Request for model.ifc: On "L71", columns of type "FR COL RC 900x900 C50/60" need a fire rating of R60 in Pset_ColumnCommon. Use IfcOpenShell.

First a look at what the model holds.

```python
import ifcopenshell
import ifcopenshell.util.element

model = ifcopenshell.open("model.ifc")
print(model.schema)
storey = next(s for s in model.by_type("IfcBuildingStorey") if s.Name == "L71")
columns = [e for e in ifcopenshell.util.element.get_decomposition(storey) if e.is_a("IfcColumn")]
seen = {}
for e in columns:
    element_type = ifcopenshell.util.element.get_type(e)
    key = (element_type.Name if element_type != e and element_type else None, ifcopenshell.util.element.get_pset(e, "Pset_ColumnCommon", "FireRating"))
    seen[key] = seen.get(key, 0) + 1
for (name, value), count in sorted(seen.items(), key=str):
    print(count, "x", name, "|", value)
```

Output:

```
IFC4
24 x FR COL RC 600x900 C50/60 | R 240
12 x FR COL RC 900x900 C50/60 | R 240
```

```python
import ifcopenshell
import ifcopenshell.api.pset
import ifcopenshell.util.element

model = ifcopenshell.open("model.ifc")

storey = next(s for s in model.by_type("IfcBuildingStorey") if s.Name == "L71")
columns = [e for e in ifcopenshell.util.element.get_decomposition(storey) if e.is_a("IfcColumn")]

count = 0
for e in columns:
    element_type = ifcopenshell.util.element.get_type(e)
    if element_type in (None, e) or element_type.Name != "FR COL RC 900x900 C50/60":
        continue
    found = ifcopenshell.util.element.get_pset(e, "Pset_ColumnCommon", should_inherit=False)
    if found:
        pset = model.by_id(found["id"])
        if len(ifcopenshell.util.element.get_elements_by_pset(pset)) > 1:
            pset = ifcopenshell.api.pset.unshare_pset(model, products=[e], pset=pset)[0]
    else:
        pset = ifcopenshell.api.pset.add_pset(model, product=e, name="Pset_ColumnCommon")
    ifcopenshell.api.pset.edit_pset(model, pset=pset, properties={"FireRating": "R60"})
    count += 1

print(count, "columns updated")

model.write("model_updated.ifc")
```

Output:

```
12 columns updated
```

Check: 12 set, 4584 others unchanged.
